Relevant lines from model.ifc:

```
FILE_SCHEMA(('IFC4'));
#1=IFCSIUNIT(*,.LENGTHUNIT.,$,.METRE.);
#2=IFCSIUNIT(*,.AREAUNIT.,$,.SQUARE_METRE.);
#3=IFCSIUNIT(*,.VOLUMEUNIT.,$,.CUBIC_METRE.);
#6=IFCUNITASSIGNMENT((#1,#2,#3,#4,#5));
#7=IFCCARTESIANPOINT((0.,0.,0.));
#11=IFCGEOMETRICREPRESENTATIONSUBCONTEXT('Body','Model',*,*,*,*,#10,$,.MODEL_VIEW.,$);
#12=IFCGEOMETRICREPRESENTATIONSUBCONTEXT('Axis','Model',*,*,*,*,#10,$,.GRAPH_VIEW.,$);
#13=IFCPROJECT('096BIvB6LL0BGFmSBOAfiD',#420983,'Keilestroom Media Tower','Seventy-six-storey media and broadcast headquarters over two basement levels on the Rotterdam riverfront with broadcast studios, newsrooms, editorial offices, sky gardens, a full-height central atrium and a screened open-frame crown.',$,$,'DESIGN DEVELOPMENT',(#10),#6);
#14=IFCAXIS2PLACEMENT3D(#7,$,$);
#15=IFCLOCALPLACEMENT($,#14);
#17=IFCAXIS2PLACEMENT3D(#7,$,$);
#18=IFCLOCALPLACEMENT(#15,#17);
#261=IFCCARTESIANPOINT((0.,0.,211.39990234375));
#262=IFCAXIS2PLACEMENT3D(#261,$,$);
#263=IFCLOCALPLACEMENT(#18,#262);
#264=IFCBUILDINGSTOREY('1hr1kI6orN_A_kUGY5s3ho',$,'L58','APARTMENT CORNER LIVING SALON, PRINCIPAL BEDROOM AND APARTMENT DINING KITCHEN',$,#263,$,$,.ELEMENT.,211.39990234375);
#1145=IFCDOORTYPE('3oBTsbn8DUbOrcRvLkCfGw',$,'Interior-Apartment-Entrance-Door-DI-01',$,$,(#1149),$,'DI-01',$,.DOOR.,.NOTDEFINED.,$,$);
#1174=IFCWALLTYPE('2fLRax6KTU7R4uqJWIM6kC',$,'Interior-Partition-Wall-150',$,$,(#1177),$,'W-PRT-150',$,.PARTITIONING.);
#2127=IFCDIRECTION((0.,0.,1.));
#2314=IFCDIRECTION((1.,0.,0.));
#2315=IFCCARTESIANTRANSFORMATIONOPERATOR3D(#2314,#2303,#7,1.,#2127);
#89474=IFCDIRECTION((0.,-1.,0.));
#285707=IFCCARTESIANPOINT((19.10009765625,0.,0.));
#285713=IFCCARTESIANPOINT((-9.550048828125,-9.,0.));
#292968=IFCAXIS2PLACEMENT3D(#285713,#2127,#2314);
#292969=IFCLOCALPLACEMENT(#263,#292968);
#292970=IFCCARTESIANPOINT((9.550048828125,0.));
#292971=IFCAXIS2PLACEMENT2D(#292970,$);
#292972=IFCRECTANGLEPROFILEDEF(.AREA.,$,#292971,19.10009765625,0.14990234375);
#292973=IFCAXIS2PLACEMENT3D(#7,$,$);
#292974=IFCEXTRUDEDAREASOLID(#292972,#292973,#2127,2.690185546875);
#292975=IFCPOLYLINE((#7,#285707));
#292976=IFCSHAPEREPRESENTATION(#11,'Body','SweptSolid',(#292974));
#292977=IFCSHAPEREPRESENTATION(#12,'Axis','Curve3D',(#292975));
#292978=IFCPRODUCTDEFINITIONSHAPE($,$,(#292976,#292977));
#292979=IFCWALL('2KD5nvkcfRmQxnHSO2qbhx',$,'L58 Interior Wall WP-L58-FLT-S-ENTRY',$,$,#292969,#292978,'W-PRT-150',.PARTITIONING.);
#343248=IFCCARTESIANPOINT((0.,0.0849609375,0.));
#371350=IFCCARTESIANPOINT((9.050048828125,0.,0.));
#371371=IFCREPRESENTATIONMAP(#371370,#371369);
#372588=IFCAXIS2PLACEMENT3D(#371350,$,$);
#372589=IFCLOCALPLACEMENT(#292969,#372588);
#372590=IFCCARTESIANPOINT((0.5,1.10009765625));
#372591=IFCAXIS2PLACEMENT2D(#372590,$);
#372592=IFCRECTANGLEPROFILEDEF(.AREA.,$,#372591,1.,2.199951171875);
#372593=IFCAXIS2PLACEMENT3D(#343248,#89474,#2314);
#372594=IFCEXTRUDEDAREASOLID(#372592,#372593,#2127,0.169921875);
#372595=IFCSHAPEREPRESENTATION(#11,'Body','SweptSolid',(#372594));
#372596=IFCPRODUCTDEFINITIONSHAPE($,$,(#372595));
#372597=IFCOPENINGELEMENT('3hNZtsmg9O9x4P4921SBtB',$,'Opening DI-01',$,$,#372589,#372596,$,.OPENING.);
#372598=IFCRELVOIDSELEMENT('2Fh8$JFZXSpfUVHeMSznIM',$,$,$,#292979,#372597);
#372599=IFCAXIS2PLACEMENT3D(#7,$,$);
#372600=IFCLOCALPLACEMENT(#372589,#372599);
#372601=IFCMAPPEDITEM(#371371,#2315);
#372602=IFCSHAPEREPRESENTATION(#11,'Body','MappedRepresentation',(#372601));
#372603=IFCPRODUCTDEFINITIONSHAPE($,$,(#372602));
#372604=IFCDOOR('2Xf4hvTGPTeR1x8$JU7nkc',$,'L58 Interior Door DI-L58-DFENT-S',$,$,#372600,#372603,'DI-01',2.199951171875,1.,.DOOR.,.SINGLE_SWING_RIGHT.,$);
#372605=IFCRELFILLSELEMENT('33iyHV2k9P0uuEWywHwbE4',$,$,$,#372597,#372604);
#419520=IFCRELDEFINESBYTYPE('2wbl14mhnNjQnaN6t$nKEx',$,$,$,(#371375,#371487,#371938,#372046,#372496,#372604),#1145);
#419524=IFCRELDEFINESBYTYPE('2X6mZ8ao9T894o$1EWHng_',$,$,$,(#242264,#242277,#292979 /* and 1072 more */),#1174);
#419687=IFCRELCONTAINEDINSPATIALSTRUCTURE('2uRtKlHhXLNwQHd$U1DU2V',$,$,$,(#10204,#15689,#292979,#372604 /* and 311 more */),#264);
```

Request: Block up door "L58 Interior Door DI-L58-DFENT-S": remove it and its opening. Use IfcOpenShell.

```python
import ifcopenshell
import ifcopenshell.api.feature
import ifcopenshell.api.root
import ifcopenshell.geom
import ifcopenshell.util.shape

model = ifcopenshell.open("model.ifc")
settings = ifcopenshell.geom.settings()


def volume(element):
    """Net volume in cubic metres, openings subtracted."""
    shape = ifcopenshell.geom.create_shape(settings, element)
    return ifcopenshell.util.shape.get_volume(shape.geometry)


door = model.by_guid("2Xf4hvTGPTeR1x8$JU7nkc")
opening = door.FillsVoids[0].RelatingOpeningElement
wall = opening.VoidsElements[0].RelatingBuildingElement
before = volume(wall)

ifcopenshell.api.root.remove_product(model, product=door)
ifcopenshell.api.feature.remove_feature(model, feature=opening)

after = volume(wall)

print(f"wall volume {before:.3f} -> {after:.3f} m3")

model.write("model_v2.ifc")
```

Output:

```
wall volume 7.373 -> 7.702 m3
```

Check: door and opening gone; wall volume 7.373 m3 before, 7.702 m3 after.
